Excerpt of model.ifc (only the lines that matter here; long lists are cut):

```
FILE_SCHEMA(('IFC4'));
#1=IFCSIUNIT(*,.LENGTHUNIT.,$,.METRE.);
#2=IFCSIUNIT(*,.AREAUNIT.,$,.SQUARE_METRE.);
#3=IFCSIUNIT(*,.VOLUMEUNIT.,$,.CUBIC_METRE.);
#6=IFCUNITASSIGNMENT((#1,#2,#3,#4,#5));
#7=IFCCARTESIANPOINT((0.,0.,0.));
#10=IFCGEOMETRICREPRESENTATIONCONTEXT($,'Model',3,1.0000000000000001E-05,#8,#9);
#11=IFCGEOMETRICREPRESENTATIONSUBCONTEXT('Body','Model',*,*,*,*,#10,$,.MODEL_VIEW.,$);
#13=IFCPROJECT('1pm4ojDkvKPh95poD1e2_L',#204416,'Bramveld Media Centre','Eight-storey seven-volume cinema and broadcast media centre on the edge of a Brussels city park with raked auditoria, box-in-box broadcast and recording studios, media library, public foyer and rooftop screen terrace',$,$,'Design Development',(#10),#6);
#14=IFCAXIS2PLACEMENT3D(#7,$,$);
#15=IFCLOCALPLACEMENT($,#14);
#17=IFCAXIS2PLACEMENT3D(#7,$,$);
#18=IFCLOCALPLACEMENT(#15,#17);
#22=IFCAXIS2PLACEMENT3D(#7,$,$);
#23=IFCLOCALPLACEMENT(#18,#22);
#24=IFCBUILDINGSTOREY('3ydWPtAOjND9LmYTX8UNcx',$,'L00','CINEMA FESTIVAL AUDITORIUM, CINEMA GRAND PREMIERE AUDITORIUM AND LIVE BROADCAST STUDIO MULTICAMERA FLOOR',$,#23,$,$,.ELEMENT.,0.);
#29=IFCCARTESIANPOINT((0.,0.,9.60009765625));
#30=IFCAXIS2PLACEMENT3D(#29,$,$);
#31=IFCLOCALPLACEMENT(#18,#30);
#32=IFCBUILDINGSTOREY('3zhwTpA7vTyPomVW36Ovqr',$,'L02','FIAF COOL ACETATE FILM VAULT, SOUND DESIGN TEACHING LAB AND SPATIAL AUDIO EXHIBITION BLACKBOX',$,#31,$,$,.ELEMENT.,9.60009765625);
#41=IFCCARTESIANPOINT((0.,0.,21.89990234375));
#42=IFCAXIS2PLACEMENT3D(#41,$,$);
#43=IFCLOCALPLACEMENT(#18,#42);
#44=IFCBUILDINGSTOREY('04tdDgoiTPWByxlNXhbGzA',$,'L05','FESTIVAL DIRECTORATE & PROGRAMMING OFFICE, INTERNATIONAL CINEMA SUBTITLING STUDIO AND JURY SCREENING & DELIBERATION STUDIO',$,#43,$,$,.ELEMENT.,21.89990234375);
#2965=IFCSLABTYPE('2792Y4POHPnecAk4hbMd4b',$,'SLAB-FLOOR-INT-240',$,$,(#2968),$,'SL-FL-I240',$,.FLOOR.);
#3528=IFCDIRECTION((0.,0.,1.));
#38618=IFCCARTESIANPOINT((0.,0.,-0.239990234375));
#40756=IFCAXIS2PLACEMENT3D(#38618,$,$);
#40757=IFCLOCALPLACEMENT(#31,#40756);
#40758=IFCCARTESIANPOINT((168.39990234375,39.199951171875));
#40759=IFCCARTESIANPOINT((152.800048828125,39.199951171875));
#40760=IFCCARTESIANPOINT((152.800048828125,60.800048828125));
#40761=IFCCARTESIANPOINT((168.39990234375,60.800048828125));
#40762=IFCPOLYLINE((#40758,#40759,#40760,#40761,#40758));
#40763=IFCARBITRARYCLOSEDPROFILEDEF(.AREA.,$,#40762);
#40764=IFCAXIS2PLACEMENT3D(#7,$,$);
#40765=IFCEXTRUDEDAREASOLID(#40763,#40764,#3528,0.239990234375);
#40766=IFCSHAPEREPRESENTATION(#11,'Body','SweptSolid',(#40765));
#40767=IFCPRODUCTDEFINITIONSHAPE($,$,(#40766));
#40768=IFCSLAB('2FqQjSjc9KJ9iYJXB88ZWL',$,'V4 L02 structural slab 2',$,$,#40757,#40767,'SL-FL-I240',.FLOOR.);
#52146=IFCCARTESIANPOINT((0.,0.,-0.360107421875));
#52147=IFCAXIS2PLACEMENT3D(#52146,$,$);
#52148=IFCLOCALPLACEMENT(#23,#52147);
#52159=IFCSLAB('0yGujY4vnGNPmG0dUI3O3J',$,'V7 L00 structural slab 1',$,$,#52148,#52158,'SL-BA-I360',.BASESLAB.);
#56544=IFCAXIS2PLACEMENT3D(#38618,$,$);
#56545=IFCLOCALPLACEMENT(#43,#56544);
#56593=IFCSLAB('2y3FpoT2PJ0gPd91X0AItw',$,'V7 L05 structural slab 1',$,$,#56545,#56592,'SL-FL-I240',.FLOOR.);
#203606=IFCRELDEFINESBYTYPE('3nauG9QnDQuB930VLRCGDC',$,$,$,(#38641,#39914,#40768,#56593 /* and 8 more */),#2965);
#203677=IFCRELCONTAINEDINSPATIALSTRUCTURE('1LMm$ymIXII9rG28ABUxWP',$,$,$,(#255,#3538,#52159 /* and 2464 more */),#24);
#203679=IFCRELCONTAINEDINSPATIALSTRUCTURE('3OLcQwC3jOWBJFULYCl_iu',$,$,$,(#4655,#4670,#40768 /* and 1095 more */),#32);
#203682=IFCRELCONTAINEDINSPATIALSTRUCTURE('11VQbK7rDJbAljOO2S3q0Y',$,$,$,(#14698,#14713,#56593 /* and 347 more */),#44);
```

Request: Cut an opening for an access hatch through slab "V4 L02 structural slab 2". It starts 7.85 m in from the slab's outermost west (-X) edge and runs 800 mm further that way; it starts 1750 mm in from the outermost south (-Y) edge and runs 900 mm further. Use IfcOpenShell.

```python
import numpy as np
import ifcopenshell
import ifcopenshell.api.feature
import ifcopenshell.api.geometry
import ifcopenshell.api.root
import ifcopenshell.geom
import ifcopenshell.util.placement
import ifcopenshell.util.representation
import ifcopenshell.util.shape
import ifcopenshell.util.unit

model = ifcopenshell.open("model.ifc")
unit_scale = ifcopenshell.util.unit.calculate_unit_scale(model)
settings = ifcopenshell.geom.settings()


def volume(element):
    """Net volume in cubic metres, openings subtracted."""
    shape = ifcopenshell.geom.create_shape(settings, element)
    return ifcopenshell.util.shape.get_volume(shape.geometry)


slab = model.by_id(40768)
before = volume(slab)

# Extent in the slab's own axes, in metres. The edges named are its -X and -Y sides.
slab_shape = ifcopenshell.geom.create_shape(settings, slab)
vertices = ifcopenshell.util.shape.get_vertices(slab_shape.geometry)
x_min, y_min, bottom = vertices.min(axis=0)
top = vertices[:, 2].max()

opening = ifcopenshell.api.root.create_entity(model, ifc_class="IfcOpeningElement", name="Access hatch opening", predefined_type="OPENING")
context = ifcopenshell.util.representation.get_context(model, "Model", "Body", "MODEL_VIEW")
width, depth = 0.8, 0.9
outline = [(0.0, 0.0), (width, 0.0), (width, depth), (0.0, depth), (0.0, 0.0)]
# Overshoot both faces by 50 mm so the cut is clean.
shape = ifcopenshell.api.geometry.add_slab_representation(
    model, context=context, depth=top - bottom + 0.1, polyline=outline
)
ifcopenshell.api.geometry.assign_representation(model, product=opening, representation=shape)

matrix = ifcopenshell.util.placement.get_local_placement(slab.ObjectPlacement)
matrix[:, 3] = matrix @ np.append(np.array([x_min + 7.85, y_min + 1.75, bottom - 0.05]) / unit_scale, 1.0)
ifcopenshell.api.geometry.edit_object_placement(model, product=opening, matrix=matrix, is_si=False)
ifcopenshell.api.feature.add_feature(model, feature=opening, element=slab)

after = volume(slab)

print(f"slab volume {before:.3f} -> {after:.3f} m3")

model.write("model_rev.ifc")
```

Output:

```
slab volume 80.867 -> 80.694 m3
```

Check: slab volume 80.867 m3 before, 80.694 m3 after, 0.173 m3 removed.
